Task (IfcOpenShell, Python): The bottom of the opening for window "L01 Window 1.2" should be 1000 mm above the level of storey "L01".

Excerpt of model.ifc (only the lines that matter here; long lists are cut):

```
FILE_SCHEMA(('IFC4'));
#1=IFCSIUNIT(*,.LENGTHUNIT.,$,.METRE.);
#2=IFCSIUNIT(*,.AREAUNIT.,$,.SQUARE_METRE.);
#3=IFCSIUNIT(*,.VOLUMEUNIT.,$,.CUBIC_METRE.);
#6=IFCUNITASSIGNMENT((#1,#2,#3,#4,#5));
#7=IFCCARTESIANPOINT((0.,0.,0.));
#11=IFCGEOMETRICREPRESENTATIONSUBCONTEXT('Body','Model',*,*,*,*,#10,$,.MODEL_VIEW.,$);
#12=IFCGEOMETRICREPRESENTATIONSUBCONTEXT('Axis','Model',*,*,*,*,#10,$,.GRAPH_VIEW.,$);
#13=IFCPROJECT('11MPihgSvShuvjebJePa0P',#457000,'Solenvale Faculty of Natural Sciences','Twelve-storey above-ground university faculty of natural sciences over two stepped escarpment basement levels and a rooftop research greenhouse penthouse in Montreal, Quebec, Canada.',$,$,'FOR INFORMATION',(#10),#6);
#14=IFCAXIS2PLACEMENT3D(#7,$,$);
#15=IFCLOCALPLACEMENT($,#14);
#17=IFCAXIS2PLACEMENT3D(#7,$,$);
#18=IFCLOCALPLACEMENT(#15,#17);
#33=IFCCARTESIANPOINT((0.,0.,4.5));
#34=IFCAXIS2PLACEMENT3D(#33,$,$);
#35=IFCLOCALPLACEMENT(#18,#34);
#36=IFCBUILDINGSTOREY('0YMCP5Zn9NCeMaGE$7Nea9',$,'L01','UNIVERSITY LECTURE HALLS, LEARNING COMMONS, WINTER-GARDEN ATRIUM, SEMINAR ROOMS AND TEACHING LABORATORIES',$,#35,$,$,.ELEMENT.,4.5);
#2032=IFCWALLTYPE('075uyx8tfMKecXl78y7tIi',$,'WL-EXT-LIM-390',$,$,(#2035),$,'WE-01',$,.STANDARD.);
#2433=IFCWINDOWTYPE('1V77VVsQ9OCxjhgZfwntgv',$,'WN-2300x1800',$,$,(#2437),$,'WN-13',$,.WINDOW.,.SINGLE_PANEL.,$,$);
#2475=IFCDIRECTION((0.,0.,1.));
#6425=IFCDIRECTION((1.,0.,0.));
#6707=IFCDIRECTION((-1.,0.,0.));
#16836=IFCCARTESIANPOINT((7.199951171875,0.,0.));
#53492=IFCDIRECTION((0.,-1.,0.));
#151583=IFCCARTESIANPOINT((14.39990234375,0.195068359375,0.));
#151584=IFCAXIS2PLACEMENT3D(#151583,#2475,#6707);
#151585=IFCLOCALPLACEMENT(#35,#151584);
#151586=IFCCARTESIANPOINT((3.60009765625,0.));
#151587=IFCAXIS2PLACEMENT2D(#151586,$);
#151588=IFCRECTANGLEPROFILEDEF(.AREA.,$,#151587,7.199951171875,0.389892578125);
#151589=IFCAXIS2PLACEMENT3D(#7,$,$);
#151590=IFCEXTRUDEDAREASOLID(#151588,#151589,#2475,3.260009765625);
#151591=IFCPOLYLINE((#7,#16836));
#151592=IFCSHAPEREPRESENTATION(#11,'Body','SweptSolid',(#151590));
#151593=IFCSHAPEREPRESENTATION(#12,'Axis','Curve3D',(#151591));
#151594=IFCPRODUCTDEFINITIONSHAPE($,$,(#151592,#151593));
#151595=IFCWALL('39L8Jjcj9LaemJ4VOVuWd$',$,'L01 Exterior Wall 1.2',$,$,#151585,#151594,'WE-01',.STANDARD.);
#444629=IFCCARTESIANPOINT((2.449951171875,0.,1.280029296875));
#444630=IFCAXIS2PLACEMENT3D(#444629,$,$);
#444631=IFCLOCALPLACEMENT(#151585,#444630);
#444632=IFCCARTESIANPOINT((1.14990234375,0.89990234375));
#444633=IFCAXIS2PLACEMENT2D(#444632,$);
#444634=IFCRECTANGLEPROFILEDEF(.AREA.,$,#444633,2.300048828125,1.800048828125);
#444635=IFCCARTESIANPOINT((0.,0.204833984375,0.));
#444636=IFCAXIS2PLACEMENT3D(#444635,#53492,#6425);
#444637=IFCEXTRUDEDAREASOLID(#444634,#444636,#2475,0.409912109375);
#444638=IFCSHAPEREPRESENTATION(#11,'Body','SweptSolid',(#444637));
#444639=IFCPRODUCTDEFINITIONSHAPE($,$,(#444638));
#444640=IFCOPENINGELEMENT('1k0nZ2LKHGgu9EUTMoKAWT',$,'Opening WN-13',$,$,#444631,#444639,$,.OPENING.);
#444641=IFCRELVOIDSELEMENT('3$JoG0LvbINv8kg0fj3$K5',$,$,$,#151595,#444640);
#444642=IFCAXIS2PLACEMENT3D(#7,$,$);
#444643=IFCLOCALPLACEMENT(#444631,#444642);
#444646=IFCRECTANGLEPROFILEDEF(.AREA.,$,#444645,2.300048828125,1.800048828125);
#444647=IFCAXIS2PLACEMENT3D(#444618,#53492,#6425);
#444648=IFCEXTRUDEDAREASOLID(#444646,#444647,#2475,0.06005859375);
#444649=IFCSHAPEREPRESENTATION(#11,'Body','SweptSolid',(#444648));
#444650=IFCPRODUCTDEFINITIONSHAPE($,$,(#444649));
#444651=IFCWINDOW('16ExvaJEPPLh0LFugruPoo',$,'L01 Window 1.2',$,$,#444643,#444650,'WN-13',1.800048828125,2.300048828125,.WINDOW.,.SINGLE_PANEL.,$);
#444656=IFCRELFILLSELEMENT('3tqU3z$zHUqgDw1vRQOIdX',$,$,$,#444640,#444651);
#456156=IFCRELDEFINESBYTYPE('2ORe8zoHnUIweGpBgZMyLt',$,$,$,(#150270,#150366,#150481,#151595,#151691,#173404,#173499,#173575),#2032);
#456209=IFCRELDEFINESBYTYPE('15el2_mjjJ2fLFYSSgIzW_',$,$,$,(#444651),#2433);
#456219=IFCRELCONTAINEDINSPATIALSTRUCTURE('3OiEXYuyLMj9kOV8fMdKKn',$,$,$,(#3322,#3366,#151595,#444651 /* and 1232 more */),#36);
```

```python
import numpy as np
import ifcopenshell
import ifcopenshell.api.geometry
import ifcopenshell.geom
import ifcopenshell.util.element
import ifcopenshell.util.placement
import ifcopenshell.util.shape
import ifcopenshell.util.unit

model = ifcopenshell.open("model.ifc")
unit_scale = ifcopenshell.util.unit.calculate_unit_scale(model)

window = model.by_id(444651)
opening = window.FillsVoids[0].RelatingOpeningElement
storey = ifcopenshell.util.element.get_container(window, ifc_class="IfcBuildingStorey")
level = ifcopenshell.util.placement.get_local_placement(storey.ObjectPlacement)[2, 3]

# The opening's origin need not be at the sill, so measure its lowest point.
shape = ifcopenshell.geom.create_shape(ifcopenshell.geom.settings(), opening)
bottom = ifcopenshell.util.shape.get_shape_bottom_elevation(shape, shape.geometry) / unit_scale
dz = level + 1.0 - bottom

shift = np.array([0.0, 0.0, dz])
# The window is placed relative to its opening, so it follows when the opening moves.
matrix = ifcopenshell.util.placement.get_local_placement(opening.ObjectPlacement)
matrix[:3, 3] += shift
ifcopenshell.api.geometry.edit_object_placement(
    model, product=opening, matrix=matrix, is_si=False, should_transform_children=True
)

print(f"moved by {dz * unit_scale:+.3f} m")

model.write("model_rev.ifc")
```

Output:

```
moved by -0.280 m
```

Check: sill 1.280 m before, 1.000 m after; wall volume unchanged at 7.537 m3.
